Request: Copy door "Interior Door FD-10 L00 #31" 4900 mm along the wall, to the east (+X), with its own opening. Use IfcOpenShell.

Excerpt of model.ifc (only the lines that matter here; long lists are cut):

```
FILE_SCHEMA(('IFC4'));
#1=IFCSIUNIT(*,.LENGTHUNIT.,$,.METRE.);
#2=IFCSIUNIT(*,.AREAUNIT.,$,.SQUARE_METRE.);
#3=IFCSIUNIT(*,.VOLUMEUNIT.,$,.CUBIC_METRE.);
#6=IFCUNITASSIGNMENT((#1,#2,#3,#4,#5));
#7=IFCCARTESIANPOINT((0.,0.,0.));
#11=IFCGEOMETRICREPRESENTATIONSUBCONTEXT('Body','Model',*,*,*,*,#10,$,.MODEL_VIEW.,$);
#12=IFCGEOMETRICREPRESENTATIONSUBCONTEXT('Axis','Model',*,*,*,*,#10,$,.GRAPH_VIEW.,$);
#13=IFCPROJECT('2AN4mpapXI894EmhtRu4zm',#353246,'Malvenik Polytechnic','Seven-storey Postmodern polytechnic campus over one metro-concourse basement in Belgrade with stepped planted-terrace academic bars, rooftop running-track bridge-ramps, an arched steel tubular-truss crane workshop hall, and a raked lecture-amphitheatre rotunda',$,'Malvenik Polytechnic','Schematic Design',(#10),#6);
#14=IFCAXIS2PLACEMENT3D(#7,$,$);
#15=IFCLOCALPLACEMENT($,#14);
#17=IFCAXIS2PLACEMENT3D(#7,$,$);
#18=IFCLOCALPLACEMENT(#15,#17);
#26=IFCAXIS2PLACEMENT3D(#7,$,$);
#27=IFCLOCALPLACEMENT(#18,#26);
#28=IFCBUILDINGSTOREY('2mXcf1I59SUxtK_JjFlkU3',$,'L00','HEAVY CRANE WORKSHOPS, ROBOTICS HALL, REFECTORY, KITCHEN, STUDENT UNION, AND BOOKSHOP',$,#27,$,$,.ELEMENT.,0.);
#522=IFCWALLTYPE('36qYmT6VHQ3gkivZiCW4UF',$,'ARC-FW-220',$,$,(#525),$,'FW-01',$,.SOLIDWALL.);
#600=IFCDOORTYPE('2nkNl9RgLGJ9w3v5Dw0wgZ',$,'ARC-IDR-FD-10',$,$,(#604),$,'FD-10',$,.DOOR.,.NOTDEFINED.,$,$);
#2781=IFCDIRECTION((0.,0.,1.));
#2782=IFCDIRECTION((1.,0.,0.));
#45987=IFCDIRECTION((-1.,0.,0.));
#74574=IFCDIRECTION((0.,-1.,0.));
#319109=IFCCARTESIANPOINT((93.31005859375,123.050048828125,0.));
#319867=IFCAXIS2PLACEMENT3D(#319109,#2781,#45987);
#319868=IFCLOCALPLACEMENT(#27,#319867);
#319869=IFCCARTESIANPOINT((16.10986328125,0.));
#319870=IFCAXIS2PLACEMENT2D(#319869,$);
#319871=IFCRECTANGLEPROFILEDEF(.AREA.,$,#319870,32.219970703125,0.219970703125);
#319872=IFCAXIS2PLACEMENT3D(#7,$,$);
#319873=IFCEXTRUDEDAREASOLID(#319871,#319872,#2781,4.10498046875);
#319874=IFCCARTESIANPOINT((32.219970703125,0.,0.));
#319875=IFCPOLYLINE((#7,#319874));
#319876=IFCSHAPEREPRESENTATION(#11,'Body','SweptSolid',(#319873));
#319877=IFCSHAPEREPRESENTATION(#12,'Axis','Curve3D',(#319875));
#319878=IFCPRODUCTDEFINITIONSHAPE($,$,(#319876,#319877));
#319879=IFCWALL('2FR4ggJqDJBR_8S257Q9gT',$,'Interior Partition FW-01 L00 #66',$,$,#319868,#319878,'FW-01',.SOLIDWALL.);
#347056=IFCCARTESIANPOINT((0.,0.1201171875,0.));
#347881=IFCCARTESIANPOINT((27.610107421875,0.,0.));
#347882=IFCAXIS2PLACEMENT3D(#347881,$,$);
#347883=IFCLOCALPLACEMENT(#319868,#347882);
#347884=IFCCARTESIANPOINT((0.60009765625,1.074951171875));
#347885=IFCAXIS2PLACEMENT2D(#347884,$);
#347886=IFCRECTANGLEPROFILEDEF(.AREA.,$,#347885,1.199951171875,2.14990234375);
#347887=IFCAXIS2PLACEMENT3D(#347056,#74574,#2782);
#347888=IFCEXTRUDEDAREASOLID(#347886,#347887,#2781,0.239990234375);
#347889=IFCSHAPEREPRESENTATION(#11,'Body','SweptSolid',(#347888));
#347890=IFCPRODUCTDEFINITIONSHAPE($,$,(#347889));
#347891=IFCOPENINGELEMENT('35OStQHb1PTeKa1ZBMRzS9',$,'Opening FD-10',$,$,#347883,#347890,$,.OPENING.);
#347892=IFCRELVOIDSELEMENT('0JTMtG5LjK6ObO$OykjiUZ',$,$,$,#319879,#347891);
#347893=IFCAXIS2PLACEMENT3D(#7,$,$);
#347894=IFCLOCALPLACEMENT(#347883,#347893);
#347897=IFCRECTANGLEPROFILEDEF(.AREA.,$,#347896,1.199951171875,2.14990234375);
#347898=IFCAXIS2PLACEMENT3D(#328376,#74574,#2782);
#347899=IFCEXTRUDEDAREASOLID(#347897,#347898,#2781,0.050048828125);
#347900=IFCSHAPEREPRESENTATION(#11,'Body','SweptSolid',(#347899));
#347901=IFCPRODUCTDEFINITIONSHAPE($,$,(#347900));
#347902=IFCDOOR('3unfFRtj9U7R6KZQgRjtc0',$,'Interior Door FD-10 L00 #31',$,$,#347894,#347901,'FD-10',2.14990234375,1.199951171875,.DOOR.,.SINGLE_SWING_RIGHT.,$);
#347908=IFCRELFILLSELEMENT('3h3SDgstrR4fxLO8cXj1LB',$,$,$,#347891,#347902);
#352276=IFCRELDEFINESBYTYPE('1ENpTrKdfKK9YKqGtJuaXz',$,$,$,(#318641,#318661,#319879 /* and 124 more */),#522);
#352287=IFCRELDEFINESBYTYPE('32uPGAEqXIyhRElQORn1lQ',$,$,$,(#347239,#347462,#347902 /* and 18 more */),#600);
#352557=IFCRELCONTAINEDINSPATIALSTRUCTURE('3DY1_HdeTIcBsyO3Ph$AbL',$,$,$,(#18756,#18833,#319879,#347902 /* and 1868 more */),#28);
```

```python
import ifcopenshell
import ifcopenshell.api.feature
import ifcopenshell.api.geometry
import ifcopenshell.api.root
import ifcopenshell.geom
import ifcopenshell.util.element
import ifcopenshell.util.placement
import ifcopenshell.util.shape

model = ifcopenshell.open("model.ifc")
settings = ifcopenshell.geom.settings()


def volume(element):
    """Net volume in cubic metres, openings subtracted."""
    shape = ifcopenshell.geom.create_shape(settings, element)
    return ifcopenshell.util.shape.get_volume(shape.geometry)


door = model.by_guid("3unfFRtj9U7R6KZQgRjtc0")
opening = door.FillsVoids[0].RelatingOpeningElement
wall = opening.VoidsElements[0].RelatingBuildingElement
before = volume(wall)
shift = ifcopenshell.util.placement.get_local_placement(wall.ObjectPlacement)[:3, 0] * -4.9

# copy_class copies the void relationship, type, container and properties, but no geometry.
new_opening = ifcopenshell.api.root.copy_class(model, product=opening)
new_opening.Representation = ifcopenshell.util.element.copy_deep(
    model, opening.Representation, exclude=["IfcGeometricRepresentationContext", "IfcRepresentationMap"]
)
new_door = ifcopenshell.api.root.copy_class(model, product=door)
new_door.Representation = ifcopenshell.util.element.copy_deep(
    model, door.Representation, exclude=["IfcGeometricRepresentationContext", "IfcRepresentationMap"]
)
new_door.Tag = None
ifcopenshell.api.feature.add_filling(model, opening=new_opening, element=new_door)

for old, new in ((opening, new_opening), (door, new_door)):
    matrix = ifcopenshell.util.placement.get_local_placement(old.ObjectPlacement)
    matrix[:3, 3] += shift
    ifcopenshell.api.geometry.edit_object_placement(model, product=new, matrix=matrix, is_si=False)

after = volume(wall)

print(f"wall volume {before:.3f} -> {after:.3f} m3")

model.write("model-out.ifc")
```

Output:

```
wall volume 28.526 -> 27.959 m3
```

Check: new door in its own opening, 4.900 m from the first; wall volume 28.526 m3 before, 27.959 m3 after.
